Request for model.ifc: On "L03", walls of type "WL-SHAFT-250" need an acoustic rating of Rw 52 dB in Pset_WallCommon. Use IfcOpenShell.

First a look at what the model holds.

```python
import ifcopenshell
import ifcopenshell.util.element

model = ifcopenshell.open("model.ifc")
print(model.schema)
storey = next(s for s in model.by_type("IfcBuildingStorey") if s.Name == "L03")
walls = [e for e in ifcopenshell.util.element.get_decomposition(storey) if e.is_a("IfcWall")]
seen = {}
for e in walls:
    element_type = ifcopenshell.util.element.get_type(e)
    key = (element_type.Name if element_type != e and element_type else None, ifcopenshell.util.element.get_pset(e, "Pset_WallCommon", "AcousticRating"))
    seen[key] = seen.get(key, 0) + 1
for (name, value), count in sorted(seen.items(), key=str):
    print(count, "x", name, "|", value)
```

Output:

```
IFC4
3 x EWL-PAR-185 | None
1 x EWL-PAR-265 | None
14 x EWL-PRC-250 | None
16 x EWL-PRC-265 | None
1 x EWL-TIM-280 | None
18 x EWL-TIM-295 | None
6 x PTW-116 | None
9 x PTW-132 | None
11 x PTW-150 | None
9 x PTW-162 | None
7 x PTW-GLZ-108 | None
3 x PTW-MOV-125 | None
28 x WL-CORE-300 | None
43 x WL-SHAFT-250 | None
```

```python
import ifcopenshell
import ifcopenshell.api.pset
import ifcopenshell.util.element

model = ifcopenshell.open("model.ifc")

storey = next(s for s in model.by_type("IfcBuildingStorey") if s.Name == "L03")
walls = [e for e in ifcopenshell.util.element.get_decomposition(storey) if e.is_a("IfcWall")]

count = 0
for e in walls:
    element_type = ifcopenshell.util.element.get_type(e)
    if element_type in (None, e) or element_type.Name != "WL-SHAFT-250":
        continue
    # add_pset returns the element's existing set when there is one.
    pset = ifcopenshell.api.pset.add_pset(model, product=e, name="Pset_WallCommon")
    ifcopenshell.api.pset.edit_pset(model, pset=pset, properties={"AcousticRating": "Rw 52 dB"})
    count += 1

print(count, "walls updated")

model.write("model_updated.ifc")
```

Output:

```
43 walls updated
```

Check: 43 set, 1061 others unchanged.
